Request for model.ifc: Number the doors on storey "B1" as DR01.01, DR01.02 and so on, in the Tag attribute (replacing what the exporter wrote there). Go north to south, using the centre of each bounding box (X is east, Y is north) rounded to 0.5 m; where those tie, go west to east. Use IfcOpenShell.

First a look at what the model holds.

```python
import ifcopenshell
import ifcopenshell.util.element
import ifcopenshell.util.placement

model = ifcopenshell.open("model.ifc")
print(model.schema)
storey = next(s for s in model.by_type("IfcBuildingStorey") if s.Name == "B1")
doors = [e for e in ifcopenshell.util.element.get_decomposition(storey) if e.is_a("IfcDoor")]
for e in sorted(doors, key=lambda e: e.id()):
    origin = ifcopenshell.util.placement.get_local_placement(e.ObjectPlacement)[:3, 3]
    print(e.id(), e.Tag, e.Name, origin.round(2) + 0.0, sep=" | ")
```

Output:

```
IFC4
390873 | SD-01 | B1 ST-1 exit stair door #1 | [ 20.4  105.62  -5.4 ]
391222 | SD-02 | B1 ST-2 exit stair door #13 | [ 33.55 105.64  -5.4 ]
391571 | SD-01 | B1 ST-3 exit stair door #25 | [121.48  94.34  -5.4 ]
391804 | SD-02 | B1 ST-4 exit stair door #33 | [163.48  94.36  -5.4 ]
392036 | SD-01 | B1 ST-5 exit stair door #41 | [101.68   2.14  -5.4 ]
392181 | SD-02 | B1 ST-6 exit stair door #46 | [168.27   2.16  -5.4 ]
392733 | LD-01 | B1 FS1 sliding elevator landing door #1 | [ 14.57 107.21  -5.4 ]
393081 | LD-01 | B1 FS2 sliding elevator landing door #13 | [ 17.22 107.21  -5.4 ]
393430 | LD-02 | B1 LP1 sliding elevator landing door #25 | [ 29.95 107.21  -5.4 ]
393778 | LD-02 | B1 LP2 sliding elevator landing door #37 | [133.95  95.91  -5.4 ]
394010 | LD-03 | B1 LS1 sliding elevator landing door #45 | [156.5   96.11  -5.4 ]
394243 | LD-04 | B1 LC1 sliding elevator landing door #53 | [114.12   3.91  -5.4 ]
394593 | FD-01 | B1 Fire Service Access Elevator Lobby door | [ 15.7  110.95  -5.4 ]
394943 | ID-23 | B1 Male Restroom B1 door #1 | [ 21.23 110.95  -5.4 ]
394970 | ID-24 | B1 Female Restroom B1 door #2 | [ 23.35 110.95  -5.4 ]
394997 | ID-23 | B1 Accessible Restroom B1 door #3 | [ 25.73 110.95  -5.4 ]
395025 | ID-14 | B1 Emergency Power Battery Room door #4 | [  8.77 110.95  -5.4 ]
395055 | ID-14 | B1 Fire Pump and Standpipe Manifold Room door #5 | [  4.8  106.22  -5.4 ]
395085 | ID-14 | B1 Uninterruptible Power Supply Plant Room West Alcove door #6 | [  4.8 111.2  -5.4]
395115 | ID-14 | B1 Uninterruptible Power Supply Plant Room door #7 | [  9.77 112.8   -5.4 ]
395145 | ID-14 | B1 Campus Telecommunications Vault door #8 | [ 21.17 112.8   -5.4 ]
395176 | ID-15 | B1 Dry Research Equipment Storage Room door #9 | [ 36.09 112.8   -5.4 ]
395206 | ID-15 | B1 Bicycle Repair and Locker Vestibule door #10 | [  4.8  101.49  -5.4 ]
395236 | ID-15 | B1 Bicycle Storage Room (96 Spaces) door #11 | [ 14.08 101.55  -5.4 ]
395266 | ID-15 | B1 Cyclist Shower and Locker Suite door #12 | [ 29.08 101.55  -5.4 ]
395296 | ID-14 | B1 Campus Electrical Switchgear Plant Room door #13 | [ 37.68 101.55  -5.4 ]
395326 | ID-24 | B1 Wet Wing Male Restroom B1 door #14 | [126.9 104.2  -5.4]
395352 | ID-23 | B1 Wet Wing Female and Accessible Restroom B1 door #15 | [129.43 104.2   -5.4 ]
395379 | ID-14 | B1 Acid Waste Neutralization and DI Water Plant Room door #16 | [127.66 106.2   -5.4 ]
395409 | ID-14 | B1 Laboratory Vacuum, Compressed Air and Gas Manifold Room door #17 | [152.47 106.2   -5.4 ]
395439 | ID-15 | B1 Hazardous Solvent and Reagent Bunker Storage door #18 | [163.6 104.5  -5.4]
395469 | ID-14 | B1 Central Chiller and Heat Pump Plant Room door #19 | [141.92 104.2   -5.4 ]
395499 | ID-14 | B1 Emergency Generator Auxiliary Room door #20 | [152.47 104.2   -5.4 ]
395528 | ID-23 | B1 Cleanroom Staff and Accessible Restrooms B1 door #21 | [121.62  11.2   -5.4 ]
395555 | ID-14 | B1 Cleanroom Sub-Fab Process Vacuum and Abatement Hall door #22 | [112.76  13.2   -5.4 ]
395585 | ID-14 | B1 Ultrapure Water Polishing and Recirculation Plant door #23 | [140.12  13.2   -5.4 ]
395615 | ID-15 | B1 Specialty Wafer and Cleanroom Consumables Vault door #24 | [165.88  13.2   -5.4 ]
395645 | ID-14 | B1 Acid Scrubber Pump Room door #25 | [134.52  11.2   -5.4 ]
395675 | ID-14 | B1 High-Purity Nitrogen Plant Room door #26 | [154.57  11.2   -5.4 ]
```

```python
import ifcopenshell
import ifcopenshell.geom
import ifcopenshell.util.element
import ifcopenshell.util.shape

model = ifcopenshell.open("model.ifc")
settings = ifcopenshell.geom.settings()
settings.set("use-world-coords", True)


def centre(element):
    shape = ifcopenshell.geom.create_shape(settings, element)
    return ifcopenshell.util.shape.get_bbox_centroid(shape.geometry)


storey = next(s for s in model.by_type("IfcBuildingStorey") if s.Name == "B1")
doors = [e for e in ifcopenshell.util.element.get_decomposition(storey) if e.is_a("IfcDoor")]

# Insertion points can sit at a corner or the storey origin, so sort by the geometry (in metres).
centres = {e: centre(e) for e in doors}
doors.sort(key=lambda e: (-round(centres[e][1] / 0.5), centres[e][0]))

for i, e in enumerate(doors, start=1):
    number = f"DR01.{i:02d}"
    e.Tag = number
    print(e.id(), number)

model.write("model_edited.ifc")
```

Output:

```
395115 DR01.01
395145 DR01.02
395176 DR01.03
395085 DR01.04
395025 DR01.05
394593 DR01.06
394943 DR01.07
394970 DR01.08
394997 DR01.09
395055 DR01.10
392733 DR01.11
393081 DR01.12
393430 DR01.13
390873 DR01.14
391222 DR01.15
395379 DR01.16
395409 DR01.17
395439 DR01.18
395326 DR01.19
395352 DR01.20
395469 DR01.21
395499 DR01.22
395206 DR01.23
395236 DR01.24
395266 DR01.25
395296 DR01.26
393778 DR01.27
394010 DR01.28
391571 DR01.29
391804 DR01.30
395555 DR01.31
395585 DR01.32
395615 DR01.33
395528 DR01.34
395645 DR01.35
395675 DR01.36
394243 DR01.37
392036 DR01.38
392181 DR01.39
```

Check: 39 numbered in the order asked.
